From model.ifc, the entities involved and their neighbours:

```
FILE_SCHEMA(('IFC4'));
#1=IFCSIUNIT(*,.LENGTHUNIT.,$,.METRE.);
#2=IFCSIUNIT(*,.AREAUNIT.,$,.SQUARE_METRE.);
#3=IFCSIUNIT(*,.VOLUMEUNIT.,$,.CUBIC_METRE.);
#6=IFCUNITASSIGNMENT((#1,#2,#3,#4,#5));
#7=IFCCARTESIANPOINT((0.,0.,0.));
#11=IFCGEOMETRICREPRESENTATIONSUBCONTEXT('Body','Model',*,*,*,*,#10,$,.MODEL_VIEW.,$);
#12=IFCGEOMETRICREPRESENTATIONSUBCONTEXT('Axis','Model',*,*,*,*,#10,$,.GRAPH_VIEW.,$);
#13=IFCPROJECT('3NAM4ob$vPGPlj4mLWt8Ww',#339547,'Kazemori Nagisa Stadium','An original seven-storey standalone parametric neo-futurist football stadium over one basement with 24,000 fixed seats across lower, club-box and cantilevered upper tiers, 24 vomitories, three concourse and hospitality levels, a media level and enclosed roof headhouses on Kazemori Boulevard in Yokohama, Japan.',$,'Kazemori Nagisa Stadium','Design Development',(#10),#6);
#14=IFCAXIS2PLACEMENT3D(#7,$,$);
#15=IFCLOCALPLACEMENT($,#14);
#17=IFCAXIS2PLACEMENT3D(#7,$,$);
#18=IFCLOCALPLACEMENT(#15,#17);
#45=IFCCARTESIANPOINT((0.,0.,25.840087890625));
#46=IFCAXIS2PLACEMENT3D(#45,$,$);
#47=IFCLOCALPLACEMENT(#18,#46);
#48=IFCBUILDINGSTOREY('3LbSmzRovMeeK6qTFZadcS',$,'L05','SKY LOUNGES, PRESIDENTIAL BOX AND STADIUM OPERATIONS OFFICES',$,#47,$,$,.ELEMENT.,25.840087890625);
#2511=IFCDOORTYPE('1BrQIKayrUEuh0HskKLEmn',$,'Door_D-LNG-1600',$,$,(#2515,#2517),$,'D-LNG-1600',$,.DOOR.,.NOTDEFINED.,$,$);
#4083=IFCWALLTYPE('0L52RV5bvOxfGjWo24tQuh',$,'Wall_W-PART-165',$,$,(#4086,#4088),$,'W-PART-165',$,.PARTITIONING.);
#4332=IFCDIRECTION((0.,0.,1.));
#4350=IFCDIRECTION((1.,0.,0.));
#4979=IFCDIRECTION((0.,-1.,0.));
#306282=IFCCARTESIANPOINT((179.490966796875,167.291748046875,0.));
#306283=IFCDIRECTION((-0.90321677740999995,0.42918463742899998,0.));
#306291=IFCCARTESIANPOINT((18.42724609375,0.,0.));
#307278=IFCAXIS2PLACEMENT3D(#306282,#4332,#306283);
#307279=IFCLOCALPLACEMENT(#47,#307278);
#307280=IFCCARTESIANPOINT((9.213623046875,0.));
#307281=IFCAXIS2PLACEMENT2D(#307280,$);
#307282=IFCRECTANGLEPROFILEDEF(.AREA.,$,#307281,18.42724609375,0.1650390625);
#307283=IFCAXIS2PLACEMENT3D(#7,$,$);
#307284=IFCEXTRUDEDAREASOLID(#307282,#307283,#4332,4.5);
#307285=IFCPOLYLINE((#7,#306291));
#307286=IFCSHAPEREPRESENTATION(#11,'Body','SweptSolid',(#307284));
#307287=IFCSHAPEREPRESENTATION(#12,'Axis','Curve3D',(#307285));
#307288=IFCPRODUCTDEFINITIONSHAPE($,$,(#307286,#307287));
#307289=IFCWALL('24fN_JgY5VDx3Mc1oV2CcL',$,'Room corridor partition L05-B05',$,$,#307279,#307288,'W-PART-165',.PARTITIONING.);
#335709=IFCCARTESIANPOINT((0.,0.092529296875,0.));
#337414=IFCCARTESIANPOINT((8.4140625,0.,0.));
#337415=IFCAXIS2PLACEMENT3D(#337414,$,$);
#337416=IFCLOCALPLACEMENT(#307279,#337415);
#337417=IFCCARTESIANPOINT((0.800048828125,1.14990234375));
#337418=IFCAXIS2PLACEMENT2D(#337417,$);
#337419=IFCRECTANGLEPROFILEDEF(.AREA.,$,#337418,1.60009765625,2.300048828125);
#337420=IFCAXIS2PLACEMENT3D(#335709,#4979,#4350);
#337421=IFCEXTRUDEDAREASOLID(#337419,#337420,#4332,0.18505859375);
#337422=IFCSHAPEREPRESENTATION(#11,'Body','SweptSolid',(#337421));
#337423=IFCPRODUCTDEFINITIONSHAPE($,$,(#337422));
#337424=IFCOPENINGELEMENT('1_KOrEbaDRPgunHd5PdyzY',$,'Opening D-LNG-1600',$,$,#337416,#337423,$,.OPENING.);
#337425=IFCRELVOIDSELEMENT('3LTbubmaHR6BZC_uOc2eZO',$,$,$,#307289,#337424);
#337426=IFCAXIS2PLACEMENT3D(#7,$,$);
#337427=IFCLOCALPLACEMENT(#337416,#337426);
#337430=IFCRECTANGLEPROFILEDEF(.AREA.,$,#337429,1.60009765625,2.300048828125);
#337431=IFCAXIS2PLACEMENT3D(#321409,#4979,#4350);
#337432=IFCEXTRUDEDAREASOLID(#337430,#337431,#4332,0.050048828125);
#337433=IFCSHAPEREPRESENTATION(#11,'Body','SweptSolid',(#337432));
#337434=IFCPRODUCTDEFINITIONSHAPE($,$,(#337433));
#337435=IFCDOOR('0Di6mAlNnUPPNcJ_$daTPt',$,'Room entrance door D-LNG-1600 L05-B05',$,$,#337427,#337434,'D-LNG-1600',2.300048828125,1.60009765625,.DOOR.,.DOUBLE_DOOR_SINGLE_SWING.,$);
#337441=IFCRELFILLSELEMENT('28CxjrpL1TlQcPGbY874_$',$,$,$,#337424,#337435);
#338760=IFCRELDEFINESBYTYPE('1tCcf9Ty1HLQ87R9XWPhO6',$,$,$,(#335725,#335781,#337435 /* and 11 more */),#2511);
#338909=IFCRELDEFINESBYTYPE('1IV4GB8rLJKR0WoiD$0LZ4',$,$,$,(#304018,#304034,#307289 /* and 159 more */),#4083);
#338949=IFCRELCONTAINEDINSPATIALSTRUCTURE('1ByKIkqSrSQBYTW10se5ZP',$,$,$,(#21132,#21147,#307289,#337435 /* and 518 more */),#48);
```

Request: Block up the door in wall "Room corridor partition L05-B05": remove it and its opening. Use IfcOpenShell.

```python
import ifcopenshell
import ifcopenshell.api.feature
import ifcopenshell.api.root
import ifcopenshell.geom
import ifcopenshell.util.shape

model = ifcopenshell.open("model.ifc")
settings = ifcopenshell.geom.settings()


def volume(element):
    """Net volume in cubic metres, openings subtracted."""
    shape = ifcopenshell.geom.create_shape(settings, element)
    return ifcopenshell.util.shape.get_volume(shape.geometry)


door = model.by_guid("0Di6mAlNnUPPNcJ_$daTPt")
opening = door.FillsVoids[0].RelatingOpeningElement
wall = opening.VoidsElements[0].RelatingBuildingElement
before = volume(wall)

ifcopenshell.api.root.remove_product(model, product=door)
ifcopenshell.api.feature.remove_feature(model, feature=opening)

after = volume(wall)

print(f"wall volume {before:.3f} -> {after:.3f} m3")

model.write("model_updated.ifc")
```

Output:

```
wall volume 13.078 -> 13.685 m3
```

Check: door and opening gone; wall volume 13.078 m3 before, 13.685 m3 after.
